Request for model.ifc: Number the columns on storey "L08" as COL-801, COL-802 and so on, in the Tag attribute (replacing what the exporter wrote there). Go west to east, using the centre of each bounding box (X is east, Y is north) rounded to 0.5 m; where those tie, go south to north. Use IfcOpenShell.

First a look at what the model holds.

```python
import ifcopenshell
import ifcopenshell.util.element
import ifcopenshell.util.placement

model = ifcopenshell.open("model.ifc")
print(model.schema)
storey = next(s for s in model.by_type("IfcBuildingStorey") if s.Name == "L08")
columns = [e for e in ifcopenshell.util.element.get_decomposition(storey) if e.is_a("IfcColumn")]
for e in sorted(columns, key=lambda e: e.id()):
    origin = ifcopenshell.util.placement.get_local_placement(e.ObjectPlacement)[:3, 3]
    print(e.id(), e.Tag, e.Name, origin.round(2) + 0.0, sep=" | ")
```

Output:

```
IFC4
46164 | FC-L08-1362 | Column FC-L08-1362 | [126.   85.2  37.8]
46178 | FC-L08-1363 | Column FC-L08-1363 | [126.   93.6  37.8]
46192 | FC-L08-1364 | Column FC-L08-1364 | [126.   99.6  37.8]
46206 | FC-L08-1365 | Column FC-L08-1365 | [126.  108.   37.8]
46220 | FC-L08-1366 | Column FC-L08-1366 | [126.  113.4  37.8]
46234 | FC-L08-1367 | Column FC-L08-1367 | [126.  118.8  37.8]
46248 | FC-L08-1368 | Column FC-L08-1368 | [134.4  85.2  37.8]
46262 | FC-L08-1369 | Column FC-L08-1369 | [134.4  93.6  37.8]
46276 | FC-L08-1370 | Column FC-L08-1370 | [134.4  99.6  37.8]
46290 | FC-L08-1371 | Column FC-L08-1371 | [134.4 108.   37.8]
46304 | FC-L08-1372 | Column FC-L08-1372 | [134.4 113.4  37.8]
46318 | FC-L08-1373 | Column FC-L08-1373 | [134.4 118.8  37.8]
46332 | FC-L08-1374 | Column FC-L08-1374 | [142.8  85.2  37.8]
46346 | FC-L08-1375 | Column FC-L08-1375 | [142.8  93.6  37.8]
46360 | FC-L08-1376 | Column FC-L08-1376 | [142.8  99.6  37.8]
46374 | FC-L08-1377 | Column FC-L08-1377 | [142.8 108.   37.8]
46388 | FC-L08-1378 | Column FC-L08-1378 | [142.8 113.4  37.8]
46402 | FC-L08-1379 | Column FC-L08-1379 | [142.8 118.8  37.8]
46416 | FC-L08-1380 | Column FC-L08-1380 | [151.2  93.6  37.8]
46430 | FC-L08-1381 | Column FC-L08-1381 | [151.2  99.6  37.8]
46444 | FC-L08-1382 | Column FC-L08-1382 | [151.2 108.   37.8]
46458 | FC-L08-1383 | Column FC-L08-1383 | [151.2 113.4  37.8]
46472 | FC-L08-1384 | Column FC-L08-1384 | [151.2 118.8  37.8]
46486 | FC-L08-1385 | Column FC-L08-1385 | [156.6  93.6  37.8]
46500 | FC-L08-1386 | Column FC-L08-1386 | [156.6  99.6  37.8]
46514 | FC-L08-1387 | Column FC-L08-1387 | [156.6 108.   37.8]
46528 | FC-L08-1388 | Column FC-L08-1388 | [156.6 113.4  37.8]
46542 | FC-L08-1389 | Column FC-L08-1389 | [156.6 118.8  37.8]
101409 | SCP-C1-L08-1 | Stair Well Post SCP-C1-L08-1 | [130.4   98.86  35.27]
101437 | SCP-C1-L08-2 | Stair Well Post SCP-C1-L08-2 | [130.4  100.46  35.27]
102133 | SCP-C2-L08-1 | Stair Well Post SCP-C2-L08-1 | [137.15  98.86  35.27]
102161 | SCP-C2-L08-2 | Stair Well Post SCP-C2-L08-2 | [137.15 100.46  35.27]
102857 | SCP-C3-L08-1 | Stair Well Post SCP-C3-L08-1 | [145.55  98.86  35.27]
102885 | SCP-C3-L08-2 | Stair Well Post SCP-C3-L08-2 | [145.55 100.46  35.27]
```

```python
import ifcopenshell
import ifcopenshell.geom
import ifcopenshell.util.element
import ifcopenshell.util.shape

model = ifcopenshell.open("model.ifc")
settings = ifcopenshell.geom.settings()
settings.set("use-world-coords", True)


def centre(element):
    shape = ifcopenshell.geom.create_shape(settings, element)
    return ifcopenshell.util.shape.get_bbox_centroid(shape.geometry)


storey = next(s for s in model.by_type("IfcBuildingStorey") if s.Name == "L08")
columns = [e for e in ifcopenshell.util.element.get_decomposition(storey) if e.is_a("IfcColumn")]

# Insertion points can sit at a corner or the storey origin, so sort by the geometry (in metres).
centres = {e: centre(e) for e in columns}
columns.sort(key=lambda e: (round(centres[e][0] / 0.5), centres[e][1]))

for i, e in enumerate(columns, start=1):
    number = f"COL-8{i:02d}"
    e.Tag = number
    print(e.id(), number)

model.write("model_updated.ifc")
```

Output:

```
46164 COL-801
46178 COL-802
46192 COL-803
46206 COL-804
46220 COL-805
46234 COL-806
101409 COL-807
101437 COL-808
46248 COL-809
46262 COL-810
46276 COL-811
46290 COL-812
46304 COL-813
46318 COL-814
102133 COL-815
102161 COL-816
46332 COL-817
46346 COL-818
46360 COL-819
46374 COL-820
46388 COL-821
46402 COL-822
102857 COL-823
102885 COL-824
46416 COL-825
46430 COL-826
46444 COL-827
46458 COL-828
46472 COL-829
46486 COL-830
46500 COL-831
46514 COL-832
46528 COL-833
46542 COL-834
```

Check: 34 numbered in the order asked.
